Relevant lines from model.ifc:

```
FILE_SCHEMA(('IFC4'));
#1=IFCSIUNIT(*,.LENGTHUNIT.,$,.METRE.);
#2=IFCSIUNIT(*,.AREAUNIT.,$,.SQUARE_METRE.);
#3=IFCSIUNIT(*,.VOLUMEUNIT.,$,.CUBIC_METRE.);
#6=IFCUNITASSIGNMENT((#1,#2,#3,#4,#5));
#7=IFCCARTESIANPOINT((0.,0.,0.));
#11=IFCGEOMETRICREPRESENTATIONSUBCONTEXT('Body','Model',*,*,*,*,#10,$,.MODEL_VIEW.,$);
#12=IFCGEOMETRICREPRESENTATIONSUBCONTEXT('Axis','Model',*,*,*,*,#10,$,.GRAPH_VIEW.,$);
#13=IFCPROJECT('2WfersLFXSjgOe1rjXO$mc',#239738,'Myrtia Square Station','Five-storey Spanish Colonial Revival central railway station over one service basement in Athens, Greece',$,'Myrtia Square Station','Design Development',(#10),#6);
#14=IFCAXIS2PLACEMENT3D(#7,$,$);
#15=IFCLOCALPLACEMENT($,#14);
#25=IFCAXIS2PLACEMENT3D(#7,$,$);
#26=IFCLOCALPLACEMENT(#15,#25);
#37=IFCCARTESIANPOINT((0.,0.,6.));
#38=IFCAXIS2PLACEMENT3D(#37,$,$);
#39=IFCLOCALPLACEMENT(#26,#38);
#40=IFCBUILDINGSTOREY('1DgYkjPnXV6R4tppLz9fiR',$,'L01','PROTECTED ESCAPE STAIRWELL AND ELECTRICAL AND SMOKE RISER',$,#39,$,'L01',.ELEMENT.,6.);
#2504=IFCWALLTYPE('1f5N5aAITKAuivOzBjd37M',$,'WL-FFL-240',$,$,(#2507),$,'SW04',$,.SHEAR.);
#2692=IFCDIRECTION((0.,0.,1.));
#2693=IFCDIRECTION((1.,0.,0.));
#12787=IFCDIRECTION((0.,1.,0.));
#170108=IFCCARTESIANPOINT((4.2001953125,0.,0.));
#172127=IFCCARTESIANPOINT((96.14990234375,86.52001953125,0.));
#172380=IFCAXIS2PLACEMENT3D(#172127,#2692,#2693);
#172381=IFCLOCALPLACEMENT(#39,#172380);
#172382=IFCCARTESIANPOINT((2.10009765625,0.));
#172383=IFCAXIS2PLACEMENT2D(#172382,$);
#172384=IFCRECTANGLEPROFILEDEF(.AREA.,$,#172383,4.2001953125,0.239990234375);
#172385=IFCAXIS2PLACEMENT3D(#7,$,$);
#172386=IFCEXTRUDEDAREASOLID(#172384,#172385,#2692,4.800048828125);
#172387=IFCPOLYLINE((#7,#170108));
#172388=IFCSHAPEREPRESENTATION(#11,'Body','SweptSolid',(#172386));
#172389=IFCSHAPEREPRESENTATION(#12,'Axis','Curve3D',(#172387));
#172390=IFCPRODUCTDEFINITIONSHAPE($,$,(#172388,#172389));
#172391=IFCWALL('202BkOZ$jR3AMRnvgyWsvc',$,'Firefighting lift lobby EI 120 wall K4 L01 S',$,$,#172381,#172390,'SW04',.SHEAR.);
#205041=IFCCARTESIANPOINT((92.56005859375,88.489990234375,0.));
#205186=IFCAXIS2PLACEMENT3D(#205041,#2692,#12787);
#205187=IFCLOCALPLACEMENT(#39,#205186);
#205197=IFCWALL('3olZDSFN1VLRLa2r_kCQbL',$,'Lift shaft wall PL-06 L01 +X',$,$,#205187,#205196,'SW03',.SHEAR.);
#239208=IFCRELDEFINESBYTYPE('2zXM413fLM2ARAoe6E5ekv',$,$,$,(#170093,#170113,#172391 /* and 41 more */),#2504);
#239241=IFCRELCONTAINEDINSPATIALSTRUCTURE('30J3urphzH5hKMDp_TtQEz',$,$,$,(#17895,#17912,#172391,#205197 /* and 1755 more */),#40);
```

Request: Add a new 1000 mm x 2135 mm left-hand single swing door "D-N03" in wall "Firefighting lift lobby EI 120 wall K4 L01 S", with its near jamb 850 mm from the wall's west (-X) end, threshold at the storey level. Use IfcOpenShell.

```python
import numpy as np
import ifcopenshell
import ifcopenshell.api.feature
import ifcopenshell.api.geometry
import ifcopenshell.api.root
import ifcopenshell.api.spatial
import ifcopenshell.geom
import ifcopenshell.util.element
import ifcopenshell.util.placement
import ifcopenshell.util.representation
import ifcopenshell.util.shape
import ifcopenshell.util.unit

model = ifcopenshell.open("model.ifc")
unit_scale = ifcopenshell.util.unit.calculate_unit_scale(model)
settings = ifcopenshell.geom.settings()


def volume(element):
    """Net volume in cubic metres, openings subtracted."""
    shape = ifcopenshell.geom.create_shape(settings, element)
    return ifcopenshell.util.shape.get_volume(shape.geometry)


wall = model.by_guid("202BkOZ$jR3AMRnvgyWsvc")
storey = ifcopenshell.util.element.get_container(wall, ifc_class="IfcBuildingStorey")
context = ifcopenshell.util.representation.get_context(model, "Model", "Body", "MODEL_VIEW")
before = volume(wall)

width, height, from_end, sill = 1, 2.135, 0.85, 0.0  # metres

# The wall runs along its own X axis, and the end named is its -X end.
wall_shape = ifcopenshell.geom.create_shape(settings, wall)
x, y, z = ifcopenshell.util.shape.get_vertices(wall_shape.geometry).T
start = x.min() + from_end
face, thickness = float(y.min()), float(y.max() - y.min())
wall_matrix = ifcopenshell.util.placement.get_local_placement(wall.ObjectPlacement)
level = ifcopenshell.util.placement.get_local_placement(storey.ObjectPlacement)[2, 3]


def in_wall(x, y):
    """Placement at x, y metres in the wall's axes, at sill height."""
    matrix = wall_matrix.copy()
    matrix[:, 3] = wall_matrix @ np.array([x / unit_scale, y / unit_scale, 0.0, 1.0])
    matrix[2, 3] = level + sill / unit_scale
    return matrix


# Opening: a box that overshoots both wall faces by 50 mm.
opening = ifcopenshell.api.root.create_entity(model, ifc_class="IfcOpeningElement", predefined_type="OPENING")
box = ifcopenshell.api.geometry.add_wall_representation(
    model, context=context, length=width, height=height, thickness=thickness + 0.1
)
ifcopenshell.api.geometry.assign_representation(model, product=opening, representation=box)
ifcopenshell.api.geometry.edit_object_placement(model, product=opening, matrix=in_wall(start, face - 0.05), is_si=False)
ifcopenshell.api.feature.add_feature(model, feature=opening, element=wall)

door = ifcopenshell.api.root.create_entity(model, ifc_class="IfcDoor", name="D-N03", predefined_type="DOOR")
door.OverallWidth, door.OverallHeight = width / unit_scale, height / unit_scale
door.OperationType = "SINGLE_SWING_LEFT"
body = ifcopenshell.api.geometry.add_door_representation(
    model,
    context=context,
    overall_width=door.OverallWidth,
    overall_height=door.OverallHeight,
    operation_type="SINGLE_SWING_LEFT",
    lining_properties={"LiningDepth": thickness / unit_scale, "ThresholdDepth": thickness / unit_scale},
)
ifcopenshell.api.geometry.assign_representation(model, product=door, representation=body)
ifcopenshell.api.spatial.assign_container(model, products=[door], relating_structure=storey)
ifcopenshell.api.feature.add_filling(model, opening=opening, element=door)

# The lining spans the wall, so the door starts at the wall face.
ifcopenshell.api.geometry.edit_object_placement(model, product=door, matrix=in_wall(start, face), is_si=False)

after = volume(wall)

print(f"wall volume {before:.3f} -> {after:.3f} m3")

model.write("model_v2.ifc")
```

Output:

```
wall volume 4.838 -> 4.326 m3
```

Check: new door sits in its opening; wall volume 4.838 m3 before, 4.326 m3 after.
